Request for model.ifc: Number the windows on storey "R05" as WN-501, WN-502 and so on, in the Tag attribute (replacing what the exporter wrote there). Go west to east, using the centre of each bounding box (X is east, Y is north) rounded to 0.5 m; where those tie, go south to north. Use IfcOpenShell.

First a look at what the model holds.

```python
import ifcopenshell
import ifcopenshell.util.element
import ifcopenshell.util.placement

model = ifcopenshell.open("model.ifc")
print(model.schema)
storey = next(s for s in model.by_type("IfcBuildingStorey") if s.Name == "R05")
windows = [e for e in ifcopenshell.util.element.get_decomposition(storey) if e.is_a("IfcWindow")]
for e in sorted(windows, key=lambda e: e.id()):
    origin = ifcopenshell.util.placement.get_local_placement(e.ObjectPlacement)[:3, 3]
    print(e.id(), e.Tag, e.Name, origin.round(2) + 0.0, sep=" | ")
```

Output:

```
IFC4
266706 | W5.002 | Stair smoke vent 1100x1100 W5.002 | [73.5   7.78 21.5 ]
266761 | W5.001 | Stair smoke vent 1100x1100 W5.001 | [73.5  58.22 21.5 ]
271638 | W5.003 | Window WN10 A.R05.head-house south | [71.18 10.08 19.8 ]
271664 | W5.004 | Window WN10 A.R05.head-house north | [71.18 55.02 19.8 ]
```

```python
import ifcopenshell
import ifcopenshell.geom
import ifcopenshell.util.element
import ifcopenshell.util.shape

model = ifcopenshell.open("model.ifc")
settings = ifcopenshell.geom.settings()
settings.set("use-world-coords", True)


def centre(element):
    shape = ifcopenshell.geom.create_shape(settings, element)
    return ifcopenshell.util.shape.get_bbox_centroid(shape.geometry)


storey = next(s for s in model.by_type("IfcBuildingStorey") if s.Name == "R05")
windows = [e for e in ifcopenshell.util.element.get_decomposition(storey) if e.is_a("IfcWindow")]

# Insertion points can sit at a corner or the storey origin, so sort by the geometry (in metres).
centres = {e: centre(e) for e in windows}
windows.sort(key=lambda e: (round(centres[e][0] / 0.5), centres[e][1]))

for i, e in enumerate(windows, start=1):
    number = f"WN-5{i:02d}"
    e.Tag = number
    print(e.id(), number)

model.write("model_updated.ifc")
```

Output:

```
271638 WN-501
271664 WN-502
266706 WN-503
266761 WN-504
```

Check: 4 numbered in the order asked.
